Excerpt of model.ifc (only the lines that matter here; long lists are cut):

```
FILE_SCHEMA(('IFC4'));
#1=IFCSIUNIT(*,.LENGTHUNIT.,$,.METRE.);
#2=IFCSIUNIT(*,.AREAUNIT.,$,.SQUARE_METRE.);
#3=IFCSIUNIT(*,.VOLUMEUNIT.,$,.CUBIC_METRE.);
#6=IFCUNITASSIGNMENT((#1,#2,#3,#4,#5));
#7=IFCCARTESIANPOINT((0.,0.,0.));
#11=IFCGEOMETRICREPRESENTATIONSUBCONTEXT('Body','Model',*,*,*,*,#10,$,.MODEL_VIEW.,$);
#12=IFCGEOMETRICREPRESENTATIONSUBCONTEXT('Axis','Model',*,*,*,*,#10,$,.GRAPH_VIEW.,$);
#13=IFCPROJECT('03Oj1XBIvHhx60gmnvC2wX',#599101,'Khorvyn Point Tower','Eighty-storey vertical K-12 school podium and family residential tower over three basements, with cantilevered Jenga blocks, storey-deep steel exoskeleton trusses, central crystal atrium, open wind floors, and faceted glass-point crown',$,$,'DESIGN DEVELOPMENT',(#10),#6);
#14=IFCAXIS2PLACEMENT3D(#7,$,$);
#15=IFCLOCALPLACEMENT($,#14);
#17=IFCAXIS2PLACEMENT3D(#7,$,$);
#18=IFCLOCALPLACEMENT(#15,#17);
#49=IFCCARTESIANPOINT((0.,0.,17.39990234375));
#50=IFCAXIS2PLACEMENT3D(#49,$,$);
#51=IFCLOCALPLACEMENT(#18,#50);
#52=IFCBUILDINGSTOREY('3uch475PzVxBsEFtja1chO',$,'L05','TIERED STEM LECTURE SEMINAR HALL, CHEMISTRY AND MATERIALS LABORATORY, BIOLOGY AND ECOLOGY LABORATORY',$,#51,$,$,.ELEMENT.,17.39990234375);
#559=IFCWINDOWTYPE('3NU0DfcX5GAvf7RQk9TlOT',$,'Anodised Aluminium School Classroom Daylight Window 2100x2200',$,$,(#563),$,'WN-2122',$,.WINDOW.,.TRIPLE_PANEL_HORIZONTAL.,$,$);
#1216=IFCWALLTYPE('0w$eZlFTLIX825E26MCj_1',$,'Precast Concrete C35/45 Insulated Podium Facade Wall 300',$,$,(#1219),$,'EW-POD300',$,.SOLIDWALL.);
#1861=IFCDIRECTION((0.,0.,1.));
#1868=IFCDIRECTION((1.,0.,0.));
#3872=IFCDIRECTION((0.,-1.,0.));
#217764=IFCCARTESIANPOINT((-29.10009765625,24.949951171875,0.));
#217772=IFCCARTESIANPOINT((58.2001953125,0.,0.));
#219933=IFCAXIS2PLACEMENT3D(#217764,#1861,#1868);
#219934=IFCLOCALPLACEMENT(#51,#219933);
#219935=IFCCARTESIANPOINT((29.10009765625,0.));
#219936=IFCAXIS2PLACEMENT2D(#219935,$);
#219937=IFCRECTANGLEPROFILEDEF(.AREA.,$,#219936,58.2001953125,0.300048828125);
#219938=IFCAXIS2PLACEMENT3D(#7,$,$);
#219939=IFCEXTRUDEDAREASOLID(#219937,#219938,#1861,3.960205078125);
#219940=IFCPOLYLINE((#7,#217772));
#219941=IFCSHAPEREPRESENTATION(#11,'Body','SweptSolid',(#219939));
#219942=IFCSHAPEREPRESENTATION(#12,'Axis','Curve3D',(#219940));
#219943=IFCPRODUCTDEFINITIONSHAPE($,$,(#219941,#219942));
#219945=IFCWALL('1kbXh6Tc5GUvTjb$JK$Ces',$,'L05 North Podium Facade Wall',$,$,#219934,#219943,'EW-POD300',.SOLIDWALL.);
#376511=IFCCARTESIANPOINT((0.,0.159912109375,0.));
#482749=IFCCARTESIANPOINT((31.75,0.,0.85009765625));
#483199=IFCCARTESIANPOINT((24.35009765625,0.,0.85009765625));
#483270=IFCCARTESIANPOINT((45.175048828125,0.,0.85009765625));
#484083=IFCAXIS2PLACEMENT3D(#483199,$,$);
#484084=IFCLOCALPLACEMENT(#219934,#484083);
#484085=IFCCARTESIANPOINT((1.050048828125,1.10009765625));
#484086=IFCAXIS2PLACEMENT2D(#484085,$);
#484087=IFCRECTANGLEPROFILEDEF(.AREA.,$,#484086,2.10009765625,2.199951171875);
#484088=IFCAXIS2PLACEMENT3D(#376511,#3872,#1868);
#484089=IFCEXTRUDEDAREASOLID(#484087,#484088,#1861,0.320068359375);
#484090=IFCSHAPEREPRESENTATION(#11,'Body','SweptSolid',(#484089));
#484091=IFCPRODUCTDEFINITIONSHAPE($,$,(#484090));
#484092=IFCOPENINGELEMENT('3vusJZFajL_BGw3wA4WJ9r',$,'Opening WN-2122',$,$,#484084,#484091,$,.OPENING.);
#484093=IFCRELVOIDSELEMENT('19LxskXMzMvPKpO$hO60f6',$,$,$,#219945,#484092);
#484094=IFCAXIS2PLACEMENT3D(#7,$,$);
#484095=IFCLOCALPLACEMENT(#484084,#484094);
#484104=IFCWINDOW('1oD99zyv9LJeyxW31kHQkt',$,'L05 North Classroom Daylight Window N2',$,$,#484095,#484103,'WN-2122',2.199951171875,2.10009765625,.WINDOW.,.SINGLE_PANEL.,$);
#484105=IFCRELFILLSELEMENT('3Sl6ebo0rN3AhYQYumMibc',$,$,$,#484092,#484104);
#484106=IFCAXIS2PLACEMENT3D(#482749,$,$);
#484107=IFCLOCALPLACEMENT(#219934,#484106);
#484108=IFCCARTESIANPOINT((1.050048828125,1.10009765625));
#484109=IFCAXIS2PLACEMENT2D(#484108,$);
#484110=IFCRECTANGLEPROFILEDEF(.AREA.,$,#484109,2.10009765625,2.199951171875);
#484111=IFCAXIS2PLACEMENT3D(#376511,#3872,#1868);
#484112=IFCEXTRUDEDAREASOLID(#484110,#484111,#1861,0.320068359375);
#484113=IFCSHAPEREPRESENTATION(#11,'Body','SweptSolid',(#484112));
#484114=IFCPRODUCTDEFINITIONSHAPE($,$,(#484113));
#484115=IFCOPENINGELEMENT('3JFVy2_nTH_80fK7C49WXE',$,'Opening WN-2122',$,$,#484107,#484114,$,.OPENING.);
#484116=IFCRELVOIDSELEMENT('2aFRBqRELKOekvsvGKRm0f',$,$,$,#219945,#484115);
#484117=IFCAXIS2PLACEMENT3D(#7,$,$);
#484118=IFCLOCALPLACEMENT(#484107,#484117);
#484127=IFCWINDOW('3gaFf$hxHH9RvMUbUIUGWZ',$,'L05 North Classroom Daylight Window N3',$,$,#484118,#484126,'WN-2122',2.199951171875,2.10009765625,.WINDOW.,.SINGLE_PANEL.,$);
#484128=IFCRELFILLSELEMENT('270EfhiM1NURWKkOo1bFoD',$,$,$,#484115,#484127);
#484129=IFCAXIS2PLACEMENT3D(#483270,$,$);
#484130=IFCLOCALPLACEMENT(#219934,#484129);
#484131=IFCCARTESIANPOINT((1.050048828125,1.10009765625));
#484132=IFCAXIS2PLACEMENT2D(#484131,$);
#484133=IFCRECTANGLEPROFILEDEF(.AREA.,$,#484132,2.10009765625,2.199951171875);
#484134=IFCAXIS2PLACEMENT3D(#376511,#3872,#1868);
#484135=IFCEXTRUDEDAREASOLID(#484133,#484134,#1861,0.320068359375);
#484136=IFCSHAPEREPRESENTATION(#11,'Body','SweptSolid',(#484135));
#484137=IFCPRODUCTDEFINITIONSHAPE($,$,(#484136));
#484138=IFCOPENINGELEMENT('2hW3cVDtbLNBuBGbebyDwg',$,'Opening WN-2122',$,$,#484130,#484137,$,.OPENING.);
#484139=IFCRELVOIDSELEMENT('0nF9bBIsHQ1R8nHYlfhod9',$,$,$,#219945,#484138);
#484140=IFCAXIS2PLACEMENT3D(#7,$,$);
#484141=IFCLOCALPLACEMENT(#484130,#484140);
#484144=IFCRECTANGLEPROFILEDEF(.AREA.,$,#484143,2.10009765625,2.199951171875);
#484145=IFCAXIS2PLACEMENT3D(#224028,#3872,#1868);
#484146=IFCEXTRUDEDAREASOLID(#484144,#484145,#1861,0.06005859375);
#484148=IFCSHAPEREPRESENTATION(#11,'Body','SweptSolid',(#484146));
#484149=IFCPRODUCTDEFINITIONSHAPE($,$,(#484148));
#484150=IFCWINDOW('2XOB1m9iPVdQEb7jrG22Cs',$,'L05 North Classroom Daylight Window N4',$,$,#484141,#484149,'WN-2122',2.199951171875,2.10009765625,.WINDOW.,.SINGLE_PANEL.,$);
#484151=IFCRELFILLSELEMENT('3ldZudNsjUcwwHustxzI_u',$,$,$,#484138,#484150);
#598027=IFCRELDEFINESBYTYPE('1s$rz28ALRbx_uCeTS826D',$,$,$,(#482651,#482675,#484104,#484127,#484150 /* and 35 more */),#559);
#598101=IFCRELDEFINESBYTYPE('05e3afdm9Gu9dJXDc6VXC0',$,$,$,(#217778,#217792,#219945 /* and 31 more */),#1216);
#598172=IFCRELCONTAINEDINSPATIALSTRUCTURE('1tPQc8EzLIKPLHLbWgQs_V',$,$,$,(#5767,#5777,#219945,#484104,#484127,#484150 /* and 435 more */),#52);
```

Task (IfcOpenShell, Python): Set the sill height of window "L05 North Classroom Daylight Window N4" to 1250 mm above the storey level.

```python
import numpy as np
import ifcopenshell
import ifcopenshell.api.geometry
import ifcopenshell.geom
import ifcopenshell.util.element
import ifcopenshell.util.placement
import ifcopenshell.util.shape
import ifcopenshell.util.unit

model = ifcopenshell.open("model.ifc")
unit_scale = ifcopenshell.util.unit.calculate_unit_scale(model)

window = model.by_id(484150)
opening = window.FillsVoids[0].RelatingOpeningElement
storey = ifcopenshell.util.element.get_container(window, ifc_class="IfcBuildingStorey")
level = ifcopenshell.util.placement.get_local_placement(storey.ObjectPlacement)[2, 3]

# The opening's origin need not be at the sill, so measure its lowest point.
shape = ifcopenshell.geom.create_shape(ifcopenshell.geom.settings(), opening)
bottom = ifcopenshell.util.shape.get_shape_bottom_elevation(shape, shape.geometry) / unit_scale
dz = level + 1.25 / unit_scale - bottom

shift = np.array([0.0, 0.0, dz])
# The window is placed relative to its opening, so it follows when the opening moves.
matrix = ifcopenshell.util.placement.get_local_placement(opening.ObjectPlacement)
matrix[:3, 3] += shift
ifcopenshell.api.geometry.edit_object_placement(
    model, product=opening, matrix=matrix, is_si=False, should_transform_children=True
)

print(f"moved by {dz * unit_scale:+.3f} m")

model.write("model_edited.ifc")
```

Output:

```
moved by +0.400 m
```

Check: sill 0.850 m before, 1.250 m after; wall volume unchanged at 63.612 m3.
